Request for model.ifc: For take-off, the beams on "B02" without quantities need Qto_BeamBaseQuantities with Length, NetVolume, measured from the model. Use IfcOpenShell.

First a look at what the model holds.

```python
import ifcopenshell
import ifcopenshell.util.element
import ifcopenshell.util.unit

model = ifcopenshell.open("model.ifc")
print(model.schema)
for unit_type in ("LENGTHUNIT", "AREAUNIT", "VOLUMEUNIT"):
    print(unit_type, ifcopenshell.util.unit.calculate_unit_scale(model, unit_type))
storey = next(s for s in model.by_type("IfcBuildingStorey") if s.Name == "B02")
beams = [e for e in ifcopenshell.util.element.get_decomposition(storey) if e.is_a("IfcBeam")]
for e in sorted(beams, key=lambda e: e.id()):
    print(e.id(), e.is_a(), e.Name, list(ifcopenshell.util.element.get_psets(e, qtos_only=True)), sep=" | ")
```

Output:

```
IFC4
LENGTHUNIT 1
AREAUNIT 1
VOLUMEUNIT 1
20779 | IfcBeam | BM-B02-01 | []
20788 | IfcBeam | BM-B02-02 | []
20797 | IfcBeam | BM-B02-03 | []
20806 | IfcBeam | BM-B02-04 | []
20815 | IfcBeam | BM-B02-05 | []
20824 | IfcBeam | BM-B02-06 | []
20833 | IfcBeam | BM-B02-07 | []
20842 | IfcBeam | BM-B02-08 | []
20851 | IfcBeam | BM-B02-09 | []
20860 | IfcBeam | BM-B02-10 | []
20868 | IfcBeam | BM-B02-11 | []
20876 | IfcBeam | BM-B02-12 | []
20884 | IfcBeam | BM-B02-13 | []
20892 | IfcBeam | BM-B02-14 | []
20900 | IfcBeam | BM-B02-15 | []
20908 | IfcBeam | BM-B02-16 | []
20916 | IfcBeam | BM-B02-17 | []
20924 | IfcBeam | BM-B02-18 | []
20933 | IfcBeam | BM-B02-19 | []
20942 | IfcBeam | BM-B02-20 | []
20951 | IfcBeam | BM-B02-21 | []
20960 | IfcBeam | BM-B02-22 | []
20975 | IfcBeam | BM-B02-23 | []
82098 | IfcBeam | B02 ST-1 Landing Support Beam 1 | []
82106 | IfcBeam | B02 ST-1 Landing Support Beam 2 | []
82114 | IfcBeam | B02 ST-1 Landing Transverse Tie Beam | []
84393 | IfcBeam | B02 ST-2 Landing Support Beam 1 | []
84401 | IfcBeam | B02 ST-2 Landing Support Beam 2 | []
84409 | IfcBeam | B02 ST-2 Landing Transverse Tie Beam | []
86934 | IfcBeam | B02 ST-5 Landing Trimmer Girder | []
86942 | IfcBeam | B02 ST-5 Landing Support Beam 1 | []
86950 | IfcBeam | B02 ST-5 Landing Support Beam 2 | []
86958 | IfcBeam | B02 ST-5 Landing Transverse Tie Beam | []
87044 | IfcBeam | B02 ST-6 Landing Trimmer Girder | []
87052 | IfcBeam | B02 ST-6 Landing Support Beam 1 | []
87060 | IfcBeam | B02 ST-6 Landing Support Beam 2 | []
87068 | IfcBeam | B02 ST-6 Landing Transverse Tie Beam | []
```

```python
import ifcopenshell
import ifcopenshell.api.pset
import ifcopenshell.geom
import ifcopenshell.util.element
import ifcopenshell.util.shape
import ifcopenshell.util.unit

model = ifcopenshell.open("model.ifc")
unit_scale = ifcopenshell.util.unit.calculate_unit_scale(model)
volume_scale = ifcopenshell.util.unit.calculate_unit_scale(model, "VOLUMEUNIT")
settings = ifcopenshell.geom.settings()

storey = next(s for s in model.by_type("IfcBuildingStorey") if s.Name == "B02")
beams = [e for e in ifcopenshell.util.element.get_decomposition(storey) if e.is_a("IfcBeam")]

for e in sorted(beams, key=lambda e: e.id()):
    if ifcopenshell.util.element.get_psets(e, qtos_only=True, should_inherit=False):
        continue
    # Geometry comes back in metres, in the element's own axes.
    shape = ifcopenshell.geom.create_shape(settings, e)
    values = {
        "Length": ifcopenshell.util.shape.get_max_xyz(shape.geometry) / unit_scale,
        "NetVolume": ifcopenshell.util.shape.get_volume(shape.geometry) / volume_scale,
    }
    qto = ifcopenshell.api.pset.add_qto(model, product=e, name="Qto_BeamBaseQuantities")
    ifcopenshell.api.pset.edit_qto(model, qto=qto, properties=values)
    print(e.id(), {k: round(v, 3) for k, v in values.items()})

model.write("model-out.ifc")
```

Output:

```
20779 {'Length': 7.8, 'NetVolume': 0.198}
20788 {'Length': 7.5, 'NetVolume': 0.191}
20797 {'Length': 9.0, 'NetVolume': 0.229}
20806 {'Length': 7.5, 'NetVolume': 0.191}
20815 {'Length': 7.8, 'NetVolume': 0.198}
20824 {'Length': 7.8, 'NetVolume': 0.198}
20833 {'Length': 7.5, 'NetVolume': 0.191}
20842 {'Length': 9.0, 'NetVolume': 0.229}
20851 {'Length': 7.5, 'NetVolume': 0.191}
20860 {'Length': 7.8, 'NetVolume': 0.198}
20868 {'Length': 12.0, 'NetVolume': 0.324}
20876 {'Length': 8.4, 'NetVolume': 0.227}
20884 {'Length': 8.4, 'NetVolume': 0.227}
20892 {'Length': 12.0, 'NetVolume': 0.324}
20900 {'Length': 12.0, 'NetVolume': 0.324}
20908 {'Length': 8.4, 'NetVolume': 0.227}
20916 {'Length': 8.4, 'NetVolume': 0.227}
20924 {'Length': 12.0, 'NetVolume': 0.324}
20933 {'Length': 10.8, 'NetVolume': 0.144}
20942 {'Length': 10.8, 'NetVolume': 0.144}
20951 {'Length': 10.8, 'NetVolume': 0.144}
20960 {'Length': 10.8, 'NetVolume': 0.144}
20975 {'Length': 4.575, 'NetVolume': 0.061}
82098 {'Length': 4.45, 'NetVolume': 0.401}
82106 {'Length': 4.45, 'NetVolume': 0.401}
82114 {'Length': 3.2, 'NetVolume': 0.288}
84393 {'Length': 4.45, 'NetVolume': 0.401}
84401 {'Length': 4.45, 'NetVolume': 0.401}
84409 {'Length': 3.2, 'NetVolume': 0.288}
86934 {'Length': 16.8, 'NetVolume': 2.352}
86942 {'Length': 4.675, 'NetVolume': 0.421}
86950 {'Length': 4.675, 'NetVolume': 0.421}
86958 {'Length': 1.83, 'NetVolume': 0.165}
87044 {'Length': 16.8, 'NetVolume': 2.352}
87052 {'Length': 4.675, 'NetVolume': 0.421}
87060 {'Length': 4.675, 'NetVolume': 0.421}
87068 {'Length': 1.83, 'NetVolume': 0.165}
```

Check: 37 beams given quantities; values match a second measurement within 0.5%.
